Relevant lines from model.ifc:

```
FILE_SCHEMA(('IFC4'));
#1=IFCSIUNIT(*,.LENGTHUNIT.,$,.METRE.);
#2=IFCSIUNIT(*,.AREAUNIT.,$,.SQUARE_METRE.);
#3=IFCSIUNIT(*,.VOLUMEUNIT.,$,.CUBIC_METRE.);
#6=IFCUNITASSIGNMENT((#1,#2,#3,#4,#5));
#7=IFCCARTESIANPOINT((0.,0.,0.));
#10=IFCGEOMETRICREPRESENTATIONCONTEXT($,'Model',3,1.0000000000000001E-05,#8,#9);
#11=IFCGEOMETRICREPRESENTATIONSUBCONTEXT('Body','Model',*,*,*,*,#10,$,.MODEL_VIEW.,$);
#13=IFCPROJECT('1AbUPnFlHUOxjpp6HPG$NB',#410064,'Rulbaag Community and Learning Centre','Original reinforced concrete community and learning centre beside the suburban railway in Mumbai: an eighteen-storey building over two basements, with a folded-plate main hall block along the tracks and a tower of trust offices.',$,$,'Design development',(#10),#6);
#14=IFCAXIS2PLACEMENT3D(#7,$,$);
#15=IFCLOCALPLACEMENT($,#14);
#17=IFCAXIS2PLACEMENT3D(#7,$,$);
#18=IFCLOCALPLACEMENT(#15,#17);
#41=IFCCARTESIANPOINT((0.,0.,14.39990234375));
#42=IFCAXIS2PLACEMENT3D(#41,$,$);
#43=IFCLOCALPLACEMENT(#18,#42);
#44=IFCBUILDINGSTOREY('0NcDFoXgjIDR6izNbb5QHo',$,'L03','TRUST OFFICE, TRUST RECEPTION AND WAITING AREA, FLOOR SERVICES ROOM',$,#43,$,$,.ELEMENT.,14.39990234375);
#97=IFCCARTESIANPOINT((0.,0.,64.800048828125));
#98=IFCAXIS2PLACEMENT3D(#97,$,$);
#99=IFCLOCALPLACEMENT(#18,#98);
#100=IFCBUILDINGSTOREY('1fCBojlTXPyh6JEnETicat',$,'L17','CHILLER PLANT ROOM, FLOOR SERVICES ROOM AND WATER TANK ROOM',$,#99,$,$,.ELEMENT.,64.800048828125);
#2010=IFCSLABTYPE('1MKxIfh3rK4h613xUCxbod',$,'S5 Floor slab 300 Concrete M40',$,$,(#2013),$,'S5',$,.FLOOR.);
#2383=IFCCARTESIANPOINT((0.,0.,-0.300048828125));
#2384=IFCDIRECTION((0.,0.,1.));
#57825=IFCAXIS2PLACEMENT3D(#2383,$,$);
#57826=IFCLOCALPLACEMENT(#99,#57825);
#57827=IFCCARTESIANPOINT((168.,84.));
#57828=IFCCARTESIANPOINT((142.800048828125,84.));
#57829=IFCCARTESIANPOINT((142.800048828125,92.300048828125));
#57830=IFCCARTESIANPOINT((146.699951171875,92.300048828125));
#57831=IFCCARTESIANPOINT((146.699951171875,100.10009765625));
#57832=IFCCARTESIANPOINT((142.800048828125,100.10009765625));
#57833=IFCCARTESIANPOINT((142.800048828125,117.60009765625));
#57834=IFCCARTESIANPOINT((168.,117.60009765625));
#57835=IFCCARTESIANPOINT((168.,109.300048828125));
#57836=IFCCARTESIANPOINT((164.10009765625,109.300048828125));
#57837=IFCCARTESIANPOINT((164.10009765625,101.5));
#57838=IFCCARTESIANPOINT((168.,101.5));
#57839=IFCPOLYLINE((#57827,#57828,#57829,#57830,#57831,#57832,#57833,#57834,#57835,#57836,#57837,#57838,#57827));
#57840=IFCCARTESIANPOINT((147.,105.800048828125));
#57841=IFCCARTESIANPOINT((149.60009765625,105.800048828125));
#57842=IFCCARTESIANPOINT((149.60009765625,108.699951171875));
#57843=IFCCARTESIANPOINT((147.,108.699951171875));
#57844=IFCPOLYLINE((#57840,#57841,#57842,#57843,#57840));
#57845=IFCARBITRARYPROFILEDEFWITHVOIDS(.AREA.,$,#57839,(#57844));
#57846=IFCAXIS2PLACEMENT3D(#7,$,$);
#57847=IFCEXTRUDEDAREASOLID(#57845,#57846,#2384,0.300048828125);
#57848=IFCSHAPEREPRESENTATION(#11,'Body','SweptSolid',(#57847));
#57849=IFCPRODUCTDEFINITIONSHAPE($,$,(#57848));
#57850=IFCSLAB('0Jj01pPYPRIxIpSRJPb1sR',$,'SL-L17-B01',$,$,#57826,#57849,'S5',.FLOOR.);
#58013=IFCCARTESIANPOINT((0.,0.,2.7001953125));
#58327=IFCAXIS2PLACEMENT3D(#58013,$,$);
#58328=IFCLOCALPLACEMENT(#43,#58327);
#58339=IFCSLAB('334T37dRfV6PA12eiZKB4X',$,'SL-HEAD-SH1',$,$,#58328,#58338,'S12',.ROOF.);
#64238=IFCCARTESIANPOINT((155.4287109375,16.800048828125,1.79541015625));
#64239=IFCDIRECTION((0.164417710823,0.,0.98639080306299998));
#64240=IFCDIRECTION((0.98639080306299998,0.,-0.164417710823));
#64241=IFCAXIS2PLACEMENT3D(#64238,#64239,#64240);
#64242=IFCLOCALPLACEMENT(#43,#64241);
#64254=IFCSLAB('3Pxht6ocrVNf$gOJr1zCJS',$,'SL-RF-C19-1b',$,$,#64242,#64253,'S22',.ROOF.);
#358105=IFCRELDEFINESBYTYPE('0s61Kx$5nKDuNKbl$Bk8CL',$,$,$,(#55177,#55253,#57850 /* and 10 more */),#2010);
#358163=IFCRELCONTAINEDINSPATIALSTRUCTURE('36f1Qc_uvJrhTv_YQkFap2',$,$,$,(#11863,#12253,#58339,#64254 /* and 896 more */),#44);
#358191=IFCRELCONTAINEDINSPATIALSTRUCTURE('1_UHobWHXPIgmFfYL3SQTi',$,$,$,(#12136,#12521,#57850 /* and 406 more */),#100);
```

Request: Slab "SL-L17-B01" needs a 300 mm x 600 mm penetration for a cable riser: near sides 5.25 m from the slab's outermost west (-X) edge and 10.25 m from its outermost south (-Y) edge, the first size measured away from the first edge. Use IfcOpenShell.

```python
import numpy as np
import ifcopenshell
import ifcopenshell.api.feature
import ifcopenshell.api.geometry
import ifcopenshell.api.root
import ifcopenshell.geom
import ifcopenshell.util.placement
import ifcopenshell.util.representation
import ifcopenshell.util.shape
import ifcopenshell.util.unit

model = ifcopenshell.open("model.ifc")
unit_scale = ifcopenshell.util.unit.calculate_unit_scale(model)
settings = ifcopenshell.geom.settings()


def volume(element):
    """Net volume in cubic metres, openings subtracted."""
    shape = ifcopenshell.geom.create_shape(settings, element)
    return ifcopenshell.util.shape.get_volume(shape.geometry)


slab = model.by_id(57850)
before = volume(slab)

# Extent in the slab's own axes, in metres. The edges named are its -X and -Y sides.
slab_shape = ifcopenshell.geom.create_shape(settings, slab)
vertices = ifcopenshell.util.shape.get_vertices(slab_shape.geometry)
x_min, y_min, bottom = vertices.min(axis=0)
top = vertices[:, 2].max()

opening = ifcopenshell.api.root.create_entity(model, ifc_class="IfcOpeningElement", name="Cable riser opening", predefined_type="OPENING")
context = ifcopenshell.util.representation.get_context(model, "Model", "Body", "MODEL_VIEW")
width, depth = 0.3, 0.6
outline = [(0.0, 0.0), (width, 0.0), (width, depth), (0.0, depth), (0.0, 0.0)]
# Overshoot both faces by 50 mm so the cut is clean.
shape = ifcopenshell.api.geometry.add_slab_representation(
    model, context=context, depth=top - bottom + 0.1, polyline=outline
)
ifcopenshell.api.geometry.assign_representation(model, product=opening, representation=shape)

matrix = ifcopenshell.util.placement.get_local_placement(slab.ObjectPlacement)
matrix[:, 3] = matrix @ np.append(np.array([x_min + 5.25, y_min + 10.25, bottom - 0.05]) / unit_scale, 1.0)
ifcopenshell.api.geometry.edit_object_placement(model, product=opening, matrix=matrix, is_si=False)
ifcopenshell.api.feature.add_feature(model, feature=opening, element=slab)

after = volume(slab)

print(f"slab volume {before:.3f} -> {after:.3f} m3")

model.write("model_rev.ifc")
```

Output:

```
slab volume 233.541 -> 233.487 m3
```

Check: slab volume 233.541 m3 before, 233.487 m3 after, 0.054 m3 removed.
